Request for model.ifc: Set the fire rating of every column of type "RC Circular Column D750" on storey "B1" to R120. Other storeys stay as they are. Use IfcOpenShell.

First a look at what the model holds.

```python
import ifcopenshell
import ifcopenshell.util.element

model = ifcopenshell.open("model.ifc")
print(model.schema)
storey = next(s for s in model.by_type("IfcBuildingStorey") if s.Name == "B1")
columns = [e for e in ifcopenshell.util.element.get_decomposition(storey) if e.is_a("IfcColumn")]
seen = {}
for e in columns:
    element_type = ifcopenshell.util.element.get_type(e)
    key = (element_type.Name if element_type != e and element_type else None, ifcopenshell.util.element.get_pset(e, "Pset_ColumnCommon", "FireRating"))
    seen[key] = seen.get(key, 0) + 1
for (name, value), count in sorted(seen.items(), key=str):
    print(count, "x", name, "|", value)
```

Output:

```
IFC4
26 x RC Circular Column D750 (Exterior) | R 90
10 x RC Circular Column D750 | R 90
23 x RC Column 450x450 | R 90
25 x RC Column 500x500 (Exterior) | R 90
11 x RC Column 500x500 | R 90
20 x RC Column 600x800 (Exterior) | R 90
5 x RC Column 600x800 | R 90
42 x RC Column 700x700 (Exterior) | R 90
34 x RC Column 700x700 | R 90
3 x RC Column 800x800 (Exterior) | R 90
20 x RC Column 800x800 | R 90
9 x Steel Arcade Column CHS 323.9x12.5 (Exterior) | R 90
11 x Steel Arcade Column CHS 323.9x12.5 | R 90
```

```python
import ifcopenshell
import ifcopenshell.api.pset
import ifcopenshell.util.element

model = ifcopenshell.open("model.ifc")

storey = next(s for s in model.by_type("IfcBuildingStorey") if s.Name == "B1")
columns = [e for e in ifcopenshell.util.element.get_decomposition(storey) if e.is_a("IfcColumn")]

count = 0
for e in columns:
    element_type = ifcopenshell.util.element.get_type(e)
    if element_type in (None, e) or element_type.Name != "RC Circular Column D750":
        continue
    # add_pset returns the element's existing set when there is one.
    pset = ifcopenshell.api.pset.add_pset(model, product=e, name="Pset_ColumnCommon")
    ifcopenshell.api.pset.edit_pset(model, pset=pset, properties={"FireRating": "R120"})
    count += 1

print(count, "columns updated")

model.write("model_edited.ifc")
```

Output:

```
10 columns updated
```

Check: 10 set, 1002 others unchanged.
